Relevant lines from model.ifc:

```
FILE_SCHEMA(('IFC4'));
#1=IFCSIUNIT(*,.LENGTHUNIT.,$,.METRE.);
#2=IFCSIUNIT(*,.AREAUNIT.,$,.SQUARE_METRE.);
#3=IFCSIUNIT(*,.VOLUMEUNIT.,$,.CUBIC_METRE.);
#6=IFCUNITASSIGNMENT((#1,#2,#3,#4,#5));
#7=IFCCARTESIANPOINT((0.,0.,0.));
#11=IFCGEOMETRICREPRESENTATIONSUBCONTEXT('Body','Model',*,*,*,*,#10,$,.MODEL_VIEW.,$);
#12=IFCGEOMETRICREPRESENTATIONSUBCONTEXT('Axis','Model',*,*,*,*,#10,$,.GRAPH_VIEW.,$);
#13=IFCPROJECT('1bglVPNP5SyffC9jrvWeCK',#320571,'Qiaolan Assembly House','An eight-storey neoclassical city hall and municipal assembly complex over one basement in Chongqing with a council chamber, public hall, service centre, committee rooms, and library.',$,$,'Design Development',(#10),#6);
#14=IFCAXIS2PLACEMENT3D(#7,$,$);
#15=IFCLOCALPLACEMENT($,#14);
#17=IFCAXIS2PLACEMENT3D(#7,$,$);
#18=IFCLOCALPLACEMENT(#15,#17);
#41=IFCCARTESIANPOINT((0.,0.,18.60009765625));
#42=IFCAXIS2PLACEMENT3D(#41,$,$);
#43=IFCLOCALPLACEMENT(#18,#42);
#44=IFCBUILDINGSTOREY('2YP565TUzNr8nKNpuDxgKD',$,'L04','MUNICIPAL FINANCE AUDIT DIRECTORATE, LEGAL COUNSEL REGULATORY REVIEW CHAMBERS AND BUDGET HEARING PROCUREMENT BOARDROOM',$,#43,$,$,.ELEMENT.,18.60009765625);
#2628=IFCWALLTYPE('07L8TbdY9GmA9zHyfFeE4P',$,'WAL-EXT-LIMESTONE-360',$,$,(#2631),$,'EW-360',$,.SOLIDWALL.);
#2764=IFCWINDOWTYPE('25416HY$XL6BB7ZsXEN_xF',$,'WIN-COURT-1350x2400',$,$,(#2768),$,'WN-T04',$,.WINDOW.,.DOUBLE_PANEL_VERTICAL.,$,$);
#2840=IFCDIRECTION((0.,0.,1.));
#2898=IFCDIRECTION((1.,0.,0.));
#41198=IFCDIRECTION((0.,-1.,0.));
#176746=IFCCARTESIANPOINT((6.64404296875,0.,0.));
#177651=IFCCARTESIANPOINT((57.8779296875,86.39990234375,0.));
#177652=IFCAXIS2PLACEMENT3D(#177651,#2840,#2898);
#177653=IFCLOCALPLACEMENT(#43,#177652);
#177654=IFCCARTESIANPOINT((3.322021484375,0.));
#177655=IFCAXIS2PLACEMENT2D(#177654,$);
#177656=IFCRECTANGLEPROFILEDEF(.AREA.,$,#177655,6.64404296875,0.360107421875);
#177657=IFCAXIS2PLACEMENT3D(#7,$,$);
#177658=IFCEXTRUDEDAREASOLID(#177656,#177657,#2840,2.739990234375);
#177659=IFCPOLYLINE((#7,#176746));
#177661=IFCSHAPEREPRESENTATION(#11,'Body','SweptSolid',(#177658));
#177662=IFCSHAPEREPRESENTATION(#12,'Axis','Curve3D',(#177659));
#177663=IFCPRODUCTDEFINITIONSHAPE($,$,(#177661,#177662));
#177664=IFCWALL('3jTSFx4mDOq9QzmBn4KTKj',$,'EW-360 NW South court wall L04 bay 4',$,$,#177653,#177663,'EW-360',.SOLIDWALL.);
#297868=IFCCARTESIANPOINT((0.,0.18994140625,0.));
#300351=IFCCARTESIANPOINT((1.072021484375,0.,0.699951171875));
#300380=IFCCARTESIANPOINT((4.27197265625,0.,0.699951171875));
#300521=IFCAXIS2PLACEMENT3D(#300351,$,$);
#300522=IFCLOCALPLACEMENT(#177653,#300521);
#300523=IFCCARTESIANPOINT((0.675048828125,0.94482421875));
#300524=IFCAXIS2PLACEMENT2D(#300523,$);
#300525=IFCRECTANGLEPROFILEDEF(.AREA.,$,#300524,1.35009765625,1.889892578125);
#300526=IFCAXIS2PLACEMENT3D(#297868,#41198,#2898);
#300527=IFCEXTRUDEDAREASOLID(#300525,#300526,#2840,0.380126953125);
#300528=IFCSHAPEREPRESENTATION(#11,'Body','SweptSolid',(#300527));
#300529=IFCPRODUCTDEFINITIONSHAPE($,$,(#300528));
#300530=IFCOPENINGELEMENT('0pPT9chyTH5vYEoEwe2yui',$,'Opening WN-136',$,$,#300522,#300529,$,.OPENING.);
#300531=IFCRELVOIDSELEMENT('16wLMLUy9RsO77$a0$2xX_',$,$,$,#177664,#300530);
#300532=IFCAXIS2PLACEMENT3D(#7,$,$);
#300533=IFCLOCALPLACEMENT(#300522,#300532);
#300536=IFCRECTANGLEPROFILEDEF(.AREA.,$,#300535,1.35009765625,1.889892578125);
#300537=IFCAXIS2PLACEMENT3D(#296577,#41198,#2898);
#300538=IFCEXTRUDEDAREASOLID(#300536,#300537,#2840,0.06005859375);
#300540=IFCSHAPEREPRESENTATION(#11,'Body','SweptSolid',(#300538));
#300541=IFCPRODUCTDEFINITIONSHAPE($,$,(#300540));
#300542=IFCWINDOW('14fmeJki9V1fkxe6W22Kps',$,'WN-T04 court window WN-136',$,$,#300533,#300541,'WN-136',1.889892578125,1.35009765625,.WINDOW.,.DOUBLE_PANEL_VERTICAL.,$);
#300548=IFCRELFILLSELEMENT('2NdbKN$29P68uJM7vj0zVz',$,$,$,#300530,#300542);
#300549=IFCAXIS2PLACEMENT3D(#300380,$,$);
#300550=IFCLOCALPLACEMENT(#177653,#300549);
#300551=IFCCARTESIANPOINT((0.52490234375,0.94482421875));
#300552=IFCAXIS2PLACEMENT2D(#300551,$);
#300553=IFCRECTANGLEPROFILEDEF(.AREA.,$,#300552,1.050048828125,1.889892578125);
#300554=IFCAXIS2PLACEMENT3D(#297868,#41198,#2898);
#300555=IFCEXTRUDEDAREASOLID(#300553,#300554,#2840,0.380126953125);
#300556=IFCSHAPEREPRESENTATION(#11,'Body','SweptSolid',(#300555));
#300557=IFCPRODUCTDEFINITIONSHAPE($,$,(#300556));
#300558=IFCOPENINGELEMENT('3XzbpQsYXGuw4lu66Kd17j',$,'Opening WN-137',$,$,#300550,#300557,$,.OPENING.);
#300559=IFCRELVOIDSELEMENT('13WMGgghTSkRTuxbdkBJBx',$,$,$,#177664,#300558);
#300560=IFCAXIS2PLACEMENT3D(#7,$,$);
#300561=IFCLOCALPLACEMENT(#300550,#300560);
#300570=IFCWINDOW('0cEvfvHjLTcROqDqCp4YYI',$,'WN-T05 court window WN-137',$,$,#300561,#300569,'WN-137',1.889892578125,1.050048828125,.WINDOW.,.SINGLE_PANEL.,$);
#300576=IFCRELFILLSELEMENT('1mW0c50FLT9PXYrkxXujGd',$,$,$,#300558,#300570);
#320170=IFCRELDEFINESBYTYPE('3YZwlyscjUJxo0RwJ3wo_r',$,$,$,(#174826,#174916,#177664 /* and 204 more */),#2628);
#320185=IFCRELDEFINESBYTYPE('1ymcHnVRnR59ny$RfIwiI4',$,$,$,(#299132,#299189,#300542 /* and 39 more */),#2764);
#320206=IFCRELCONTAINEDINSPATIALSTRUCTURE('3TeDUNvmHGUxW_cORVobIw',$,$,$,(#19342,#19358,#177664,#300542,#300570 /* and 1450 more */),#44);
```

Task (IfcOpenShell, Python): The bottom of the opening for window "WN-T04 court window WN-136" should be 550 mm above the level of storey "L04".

```python
import numpy as np
import ifcopenshell
import ifcopenshell.api.geometry
import ifcopenshell.geom
import ifcopenshell.util.element
import ifcopenshell.util.placement
import ifcopenshell.util.shape
import ifcopenshell.util.unit

model = ifcopenshell.open("model.ifc")
unit_scale = ifcopenshell.util.unit.calculate_unit_scale(model)

window = model.by_id(300542)
opening = window.FillsVoids[0].RelatingOpeningElement
storey = ifcopenshell.util.element.get_container(window, ifc_class="IfcBuildingStorey")
level = ifcopenshell.util.placement.get_local_placement(storey.ObjectPlacement)[2, 3]

# The opening's origin need not be at the sill, so measure its lowest point.
shape = ifcopenshell.geom.create_shape(ifcopenshell.geom.settings(), opening)
bottom = ifcopenshell.util.shape.get_shape_bottom_elevation(shape, shape.geometry) / unit_scale
dz = level + 0.55 / unit_scale - bottom

shift = np.array([0.0, 0.0, dz])
# The window is placed relative to its opening, so it follows when the opening moves.
matrix = ifcopenshell.util.placement.get_local_placement(opening.ObjectPlacement)
matrix[:3, 3] += shift
ifcopenshell.api.geometry.edit_object_placement(
    model, product=opening, matrix=matrix, is_si=False, should_transform_children=True
)

print(f"moved by {dz * unit_scale:+.3f} m")

model.write("model_v2.ifc")
```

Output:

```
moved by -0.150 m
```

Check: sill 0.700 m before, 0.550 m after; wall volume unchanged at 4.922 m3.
